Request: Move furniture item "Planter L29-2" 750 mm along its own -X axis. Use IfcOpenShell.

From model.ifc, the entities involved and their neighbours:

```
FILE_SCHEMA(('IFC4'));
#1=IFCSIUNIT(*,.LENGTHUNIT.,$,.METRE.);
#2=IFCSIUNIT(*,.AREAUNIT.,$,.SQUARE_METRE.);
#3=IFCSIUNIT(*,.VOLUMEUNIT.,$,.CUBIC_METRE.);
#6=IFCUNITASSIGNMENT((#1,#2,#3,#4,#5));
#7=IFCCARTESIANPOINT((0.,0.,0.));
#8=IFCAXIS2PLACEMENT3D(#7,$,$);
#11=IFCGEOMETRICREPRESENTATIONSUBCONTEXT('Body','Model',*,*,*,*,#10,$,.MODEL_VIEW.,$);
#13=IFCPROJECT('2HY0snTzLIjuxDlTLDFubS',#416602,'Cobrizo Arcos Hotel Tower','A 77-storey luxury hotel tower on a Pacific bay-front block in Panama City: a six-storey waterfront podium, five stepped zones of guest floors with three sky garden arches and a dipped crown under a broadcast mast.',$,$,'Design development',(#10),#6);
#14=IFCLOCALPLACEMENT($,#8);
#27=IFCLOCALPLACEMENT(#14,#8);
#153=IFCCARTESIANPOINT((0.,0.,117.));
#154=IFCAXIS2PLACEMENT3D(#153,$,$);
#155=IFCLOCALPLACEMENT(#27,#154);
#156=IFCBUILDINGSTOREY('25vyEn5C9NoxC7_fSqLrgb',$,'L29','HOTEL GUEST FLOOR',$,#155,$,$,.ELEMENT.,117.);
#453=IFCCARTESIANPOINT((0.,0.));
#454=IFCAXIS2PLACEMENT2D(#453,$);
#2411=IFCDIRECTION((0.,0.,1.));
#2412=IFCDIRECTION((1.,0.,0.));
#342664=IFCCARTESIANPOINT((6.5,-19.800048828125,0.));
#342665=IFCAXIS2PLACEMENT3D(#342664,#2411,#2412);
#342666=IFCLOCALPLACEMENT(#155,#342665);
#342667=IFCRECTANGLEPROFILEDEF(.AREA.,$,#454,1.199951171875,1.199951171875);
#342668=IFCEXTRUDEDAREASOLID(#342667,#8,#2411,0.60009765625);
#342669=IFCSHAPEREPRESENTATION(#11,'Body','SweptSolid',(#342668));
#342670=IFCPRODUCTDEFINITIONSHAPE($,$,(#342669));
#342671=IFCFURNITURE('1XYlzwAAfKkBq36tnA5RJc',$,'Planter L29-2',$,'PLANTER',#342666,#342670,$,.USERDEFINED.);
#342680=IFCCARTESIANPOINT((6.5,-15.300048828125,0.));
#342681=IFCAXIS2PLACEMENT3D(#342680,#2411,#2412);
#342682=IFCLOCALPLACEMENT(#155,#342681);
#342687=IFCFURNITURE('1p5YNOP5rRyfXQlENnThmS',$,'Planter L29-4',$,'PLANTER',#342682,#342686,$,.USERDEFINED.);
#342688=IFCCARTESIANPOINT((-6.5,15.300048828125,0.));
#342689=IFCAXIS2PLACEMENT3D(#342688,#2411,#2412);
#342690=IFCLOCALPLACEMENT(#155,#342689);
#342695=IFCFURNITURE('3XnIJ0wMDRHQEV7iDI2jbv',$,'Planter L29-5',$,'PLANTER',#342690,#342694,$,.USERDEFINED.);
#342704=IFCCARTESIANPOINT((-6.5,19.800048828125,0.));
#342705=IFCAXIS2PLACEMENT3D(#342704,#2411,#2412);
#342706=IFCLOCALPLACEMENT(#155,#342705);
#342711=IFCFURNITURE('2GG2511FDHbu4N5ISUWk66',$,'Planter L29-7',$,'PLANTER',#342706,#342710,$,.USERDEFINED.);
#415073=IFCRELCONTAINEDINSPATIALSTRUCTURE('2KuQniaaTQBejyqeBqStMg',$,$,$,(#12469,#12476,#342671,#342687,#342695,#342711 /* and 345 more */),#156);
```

```python
import ifcopenshell
import ifcopenshell.api.geometry
import ifcopenshell.util.placement

model = ifcopenshell.open("model.ifc")

item = model.by_guid("1XYlzwAAfKkBq36tnA5RJc")
matrix = ifcopenshell.util.placement.get_local_placement(item.ObjectPlacement)
matrix[:3, 3] -= matrix[:3, 0] * 0.75
ifcopenshell.api.geometry.edit_object_placement(model, product=item, matrix=matrix, is_si=False)

print(ifcopenshell.util.placement.get_local_placement(item.ObjectPlacement).round(3) + 0.0)

model.write("model_edited.ifc")
```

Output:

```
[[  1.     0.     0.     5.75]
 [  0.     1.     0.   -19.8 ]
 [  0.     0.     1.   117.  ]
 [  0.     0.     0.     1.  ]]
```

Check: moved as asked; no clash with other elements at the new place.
